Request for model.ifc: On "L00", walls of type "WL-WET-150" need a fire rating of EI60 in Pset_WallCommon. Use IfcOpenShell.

First a look at what the model holds.

```python
import ifcopenshell
import ifcopenshell.util.element

model = ifcopenshell.open("model.ifc")
print(model.schema)
storey = next(s for s in model.by_type("IfcBuildingStorey") if s.Name == "L00")
walls = [e for e in ifcopenshell.util.element.get_decomposition(storey) if e.is_a("IfcWall")]
seen = {}
for e in walls:
    element_type = ifcopenshell.util.element.get_type(e)
    key = (element_type.Name if element_type != e and element_type else None, ifcopenshell.util.element.get_pset(e, "Pset_WallCommon", "FireRating"))
    seen[key] = seen.get(key, 0) + 1
for (name, value), count in sorted(seen.items(), key=str):
    print(count, "x", name, "|", value)
```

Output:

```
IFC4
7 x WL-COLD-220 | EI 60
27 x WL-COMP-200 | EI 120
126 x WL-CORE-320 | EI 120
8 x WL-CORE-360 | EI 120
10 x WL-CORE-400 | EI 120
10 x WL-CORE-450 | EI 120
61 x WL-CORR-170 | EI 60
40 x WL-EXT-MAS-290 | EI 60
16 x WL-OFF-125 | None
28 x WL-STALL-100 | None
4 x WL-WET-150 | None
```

```python
import ifcopenshell
import ifcopenshell.api.pset
import ifcopenshell.util.element

model = ifcopenshell.open("model.ifc")

storey = next(s for s in model.by_type("IfcBuildingStorey") if s.Name == "L00")
walls = [e for e in ifcopenshell.util.element.get_decomposition(storey) if e.is_a("IfcWall")]

count = 0
for e in walls:
    element_type = ifcopenshell.util.element.get_type(e)
    if element_type in (None, e) or element_type.Name != "WL-WET-150":
        continue
    # add_pset returns the element's existing set when there is one.
    pset = ifcopenshell.api.pset.add_pset(model, product=e, name="Pset_WallCommon")
    ifcopenshell.api.pset.edit_pset(model, pset=pset, properties={"FireRating": "EI60"})
    count += 1

print(count, "walls updated")

model.write("model_updated.ifc")
```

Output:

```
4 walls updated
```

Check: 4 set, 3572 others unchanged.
